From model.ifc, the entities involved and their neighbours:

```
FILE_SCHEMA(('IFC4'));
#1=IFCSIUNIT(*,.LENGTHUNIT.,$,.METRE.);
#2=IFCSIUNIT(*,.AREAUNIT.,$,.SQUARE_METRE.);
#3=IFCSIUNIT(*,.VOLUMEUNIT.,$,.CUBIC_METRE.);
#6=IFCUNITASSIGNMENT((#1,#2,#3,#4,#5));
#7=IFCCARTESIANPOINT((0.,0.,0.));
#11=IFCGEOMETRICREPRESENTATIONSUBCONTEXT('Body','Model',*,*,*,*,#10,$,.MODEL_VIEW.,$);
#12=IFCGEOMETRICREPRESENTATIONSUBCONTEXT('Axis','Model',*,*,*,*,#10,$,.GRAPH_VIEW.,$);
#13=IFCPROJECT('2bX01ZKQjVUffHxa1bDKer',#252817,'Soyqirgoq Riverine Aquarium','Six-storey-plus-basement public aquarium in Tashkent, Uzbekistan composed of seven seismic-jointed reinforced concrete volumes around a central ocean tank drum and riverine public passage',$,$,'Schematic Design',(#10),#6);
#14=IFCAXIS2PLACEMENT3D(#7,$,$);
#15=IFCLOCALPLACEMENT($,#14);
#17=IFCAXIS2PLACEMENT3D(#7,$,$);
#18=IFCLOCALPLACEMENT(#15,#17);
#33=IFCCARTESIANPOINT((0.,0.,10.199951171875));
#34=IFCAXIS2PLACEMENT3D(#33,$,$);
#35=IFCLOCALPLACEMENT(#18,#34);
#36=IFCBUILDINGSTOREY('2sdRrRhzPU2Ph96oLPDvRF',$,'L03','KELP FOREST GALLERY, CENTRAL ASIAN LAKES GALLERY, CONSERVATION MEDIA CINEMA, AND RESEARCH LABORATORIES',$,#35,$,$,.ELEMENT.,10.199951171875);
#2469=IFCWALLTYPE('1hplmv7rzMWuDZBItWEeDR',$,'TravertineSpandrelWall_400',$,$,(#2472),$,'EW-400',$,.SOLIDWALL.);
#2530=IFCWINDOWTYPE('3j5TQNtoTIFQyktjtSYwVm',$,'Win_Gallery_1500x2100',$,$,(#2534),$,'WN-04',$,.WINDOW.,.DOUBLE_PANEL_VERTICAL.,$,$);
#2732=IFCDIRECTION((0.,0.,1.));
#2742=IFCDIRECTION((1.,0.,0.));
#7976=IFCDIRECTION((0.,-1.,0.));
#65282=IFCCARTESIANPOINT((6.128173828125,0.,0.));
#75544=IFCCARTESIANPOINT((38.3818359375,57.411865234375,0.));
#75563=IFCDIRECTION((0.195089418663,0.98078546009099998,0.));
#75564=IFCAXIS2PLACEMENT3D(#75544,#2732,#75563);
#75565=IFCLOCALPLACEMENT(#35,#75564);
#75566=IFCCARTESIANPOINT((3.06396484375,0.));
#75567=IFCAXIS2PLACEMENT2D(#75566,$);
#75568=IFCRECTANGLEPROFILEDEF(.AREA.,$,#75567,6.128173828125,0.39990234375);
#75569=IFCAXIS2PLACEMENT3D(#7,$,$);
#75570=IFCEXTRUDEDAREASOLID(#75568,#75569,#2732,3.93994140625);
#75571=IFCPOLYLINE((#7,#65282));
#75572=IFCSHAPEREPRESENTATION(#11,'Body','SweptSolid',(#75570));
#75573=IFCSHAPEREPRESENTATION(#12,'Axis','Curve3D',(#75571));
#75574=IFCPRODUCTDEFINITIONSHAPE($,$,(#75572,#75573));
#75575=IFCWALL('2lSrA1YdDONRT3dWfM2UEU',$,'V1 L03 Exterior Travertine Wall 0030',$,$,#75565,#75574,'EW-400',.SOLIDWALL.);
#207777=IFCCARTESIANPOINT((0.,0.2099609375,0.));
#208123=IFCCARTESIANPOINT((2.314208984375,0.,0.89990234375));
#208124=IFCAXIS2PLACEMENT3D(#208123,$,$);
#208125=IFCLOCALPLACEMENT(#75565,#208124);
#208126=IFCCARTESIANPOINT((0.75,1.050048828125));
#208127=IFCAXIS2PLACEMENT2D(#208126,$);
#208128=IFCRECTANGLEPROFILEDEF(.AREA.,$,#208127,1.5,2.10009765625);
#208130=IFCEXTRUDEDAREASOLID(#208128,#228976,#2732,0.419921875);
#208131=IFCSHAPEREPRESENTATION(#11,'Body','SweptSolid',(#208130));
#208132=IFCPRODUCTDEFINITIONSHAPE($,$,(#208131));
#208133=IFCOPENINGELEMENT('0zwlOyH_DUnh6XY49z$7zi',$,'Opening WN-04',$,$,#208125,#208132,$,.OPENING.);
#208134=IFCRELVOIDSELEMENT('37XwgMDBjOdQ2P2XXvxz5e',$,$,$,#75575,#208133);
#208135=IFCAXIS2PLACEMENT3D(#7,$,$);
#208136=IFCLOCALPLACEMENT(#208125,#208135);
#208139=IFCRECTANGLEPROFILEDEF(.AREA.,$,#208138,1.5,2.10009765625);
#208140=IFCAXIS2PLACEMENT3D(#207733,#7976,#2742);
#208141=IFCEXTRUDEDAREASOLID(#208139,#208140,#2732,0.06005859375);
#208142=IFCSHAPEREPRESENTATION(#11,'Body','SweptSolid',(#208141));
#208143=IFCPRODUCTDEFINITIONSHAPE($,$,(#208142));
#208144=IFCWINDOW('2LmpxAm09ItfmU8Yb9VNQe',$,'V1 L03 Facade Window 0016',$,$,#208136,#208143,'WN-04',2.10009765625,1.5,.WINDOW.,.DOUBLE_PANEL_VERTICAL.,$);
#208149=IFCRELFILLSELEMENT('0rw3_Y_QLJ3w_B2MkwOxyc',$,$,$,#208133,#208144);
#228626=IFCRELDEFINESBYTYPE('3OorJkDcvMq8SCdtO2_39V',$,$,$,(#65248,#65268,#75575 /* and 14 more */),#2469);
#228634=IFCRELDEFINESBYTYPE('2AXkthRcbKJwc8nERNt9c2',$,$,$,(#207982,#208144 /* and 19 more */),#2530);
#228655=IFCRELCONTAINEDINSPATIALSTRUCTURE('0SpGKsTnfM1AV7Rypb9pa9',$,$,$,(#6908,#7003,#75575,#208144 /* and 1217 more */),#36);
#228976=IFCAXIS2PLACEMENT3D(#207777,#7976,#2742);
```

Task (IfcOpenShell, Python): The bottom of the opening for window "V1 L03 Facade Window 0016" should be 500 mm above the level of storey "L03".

```python
import numpy as np
import ifcopenshell
import ifcopenshell.api.geometry
import ifcopenshell.geom
import ifcopenshell.util.element
import ifcopenshell.util.placement
import ifcopenshell.util.shape
import ifcopenshell.util.unit

model = ifcopenshell.open("model.ifc")
unit_scale = ifcopenshell.util.unit.calculate_unit_scale(model)

window = model.by_guid("2LmpxAm09ItfmU8Yb9VNQe")
opening = window.FillsVoids[0].RelatingOpeningElement
storey = ifcopenshell.util.element.get_container(window, ifc_class="IfcBuildingStorey")
level = ifcopenshell.util.placement.get_local_placement(storey.ObjectPlacement)[2, 3]

# The opening's origin need not be at the sill, so measure its lowest point.
shape = ifcopenshell.geom.create_shape(ifcopenshell.geom.settings(), opening)
bottom = ifcopenshell.util.shape.get_shape_bottom_elevation(shape, shape.geometry) / unit_scale
dz = level + 0.5 / unit_scale - bottom

shift = np.array([0.0, 0.0, dz])
# The window is placed relative to its opening, so it follows when the opening moves.
matrix = ifcopenshell.util.placement.get_local_placement(opening.ObjectPlacement)
matrix[:3, 3] += shift
ifcopenshell.api.geometry.edit_object_placement(
    model, product=opening, matrix=matrix, is_si=False, should_transform_children=True
)

print(f"moved by {dz * unit_scale:+.3f} m")

model.write("model-out.ifc")
```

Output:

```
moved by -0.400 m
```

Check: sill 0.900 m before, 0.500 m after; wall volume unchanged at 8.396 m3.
